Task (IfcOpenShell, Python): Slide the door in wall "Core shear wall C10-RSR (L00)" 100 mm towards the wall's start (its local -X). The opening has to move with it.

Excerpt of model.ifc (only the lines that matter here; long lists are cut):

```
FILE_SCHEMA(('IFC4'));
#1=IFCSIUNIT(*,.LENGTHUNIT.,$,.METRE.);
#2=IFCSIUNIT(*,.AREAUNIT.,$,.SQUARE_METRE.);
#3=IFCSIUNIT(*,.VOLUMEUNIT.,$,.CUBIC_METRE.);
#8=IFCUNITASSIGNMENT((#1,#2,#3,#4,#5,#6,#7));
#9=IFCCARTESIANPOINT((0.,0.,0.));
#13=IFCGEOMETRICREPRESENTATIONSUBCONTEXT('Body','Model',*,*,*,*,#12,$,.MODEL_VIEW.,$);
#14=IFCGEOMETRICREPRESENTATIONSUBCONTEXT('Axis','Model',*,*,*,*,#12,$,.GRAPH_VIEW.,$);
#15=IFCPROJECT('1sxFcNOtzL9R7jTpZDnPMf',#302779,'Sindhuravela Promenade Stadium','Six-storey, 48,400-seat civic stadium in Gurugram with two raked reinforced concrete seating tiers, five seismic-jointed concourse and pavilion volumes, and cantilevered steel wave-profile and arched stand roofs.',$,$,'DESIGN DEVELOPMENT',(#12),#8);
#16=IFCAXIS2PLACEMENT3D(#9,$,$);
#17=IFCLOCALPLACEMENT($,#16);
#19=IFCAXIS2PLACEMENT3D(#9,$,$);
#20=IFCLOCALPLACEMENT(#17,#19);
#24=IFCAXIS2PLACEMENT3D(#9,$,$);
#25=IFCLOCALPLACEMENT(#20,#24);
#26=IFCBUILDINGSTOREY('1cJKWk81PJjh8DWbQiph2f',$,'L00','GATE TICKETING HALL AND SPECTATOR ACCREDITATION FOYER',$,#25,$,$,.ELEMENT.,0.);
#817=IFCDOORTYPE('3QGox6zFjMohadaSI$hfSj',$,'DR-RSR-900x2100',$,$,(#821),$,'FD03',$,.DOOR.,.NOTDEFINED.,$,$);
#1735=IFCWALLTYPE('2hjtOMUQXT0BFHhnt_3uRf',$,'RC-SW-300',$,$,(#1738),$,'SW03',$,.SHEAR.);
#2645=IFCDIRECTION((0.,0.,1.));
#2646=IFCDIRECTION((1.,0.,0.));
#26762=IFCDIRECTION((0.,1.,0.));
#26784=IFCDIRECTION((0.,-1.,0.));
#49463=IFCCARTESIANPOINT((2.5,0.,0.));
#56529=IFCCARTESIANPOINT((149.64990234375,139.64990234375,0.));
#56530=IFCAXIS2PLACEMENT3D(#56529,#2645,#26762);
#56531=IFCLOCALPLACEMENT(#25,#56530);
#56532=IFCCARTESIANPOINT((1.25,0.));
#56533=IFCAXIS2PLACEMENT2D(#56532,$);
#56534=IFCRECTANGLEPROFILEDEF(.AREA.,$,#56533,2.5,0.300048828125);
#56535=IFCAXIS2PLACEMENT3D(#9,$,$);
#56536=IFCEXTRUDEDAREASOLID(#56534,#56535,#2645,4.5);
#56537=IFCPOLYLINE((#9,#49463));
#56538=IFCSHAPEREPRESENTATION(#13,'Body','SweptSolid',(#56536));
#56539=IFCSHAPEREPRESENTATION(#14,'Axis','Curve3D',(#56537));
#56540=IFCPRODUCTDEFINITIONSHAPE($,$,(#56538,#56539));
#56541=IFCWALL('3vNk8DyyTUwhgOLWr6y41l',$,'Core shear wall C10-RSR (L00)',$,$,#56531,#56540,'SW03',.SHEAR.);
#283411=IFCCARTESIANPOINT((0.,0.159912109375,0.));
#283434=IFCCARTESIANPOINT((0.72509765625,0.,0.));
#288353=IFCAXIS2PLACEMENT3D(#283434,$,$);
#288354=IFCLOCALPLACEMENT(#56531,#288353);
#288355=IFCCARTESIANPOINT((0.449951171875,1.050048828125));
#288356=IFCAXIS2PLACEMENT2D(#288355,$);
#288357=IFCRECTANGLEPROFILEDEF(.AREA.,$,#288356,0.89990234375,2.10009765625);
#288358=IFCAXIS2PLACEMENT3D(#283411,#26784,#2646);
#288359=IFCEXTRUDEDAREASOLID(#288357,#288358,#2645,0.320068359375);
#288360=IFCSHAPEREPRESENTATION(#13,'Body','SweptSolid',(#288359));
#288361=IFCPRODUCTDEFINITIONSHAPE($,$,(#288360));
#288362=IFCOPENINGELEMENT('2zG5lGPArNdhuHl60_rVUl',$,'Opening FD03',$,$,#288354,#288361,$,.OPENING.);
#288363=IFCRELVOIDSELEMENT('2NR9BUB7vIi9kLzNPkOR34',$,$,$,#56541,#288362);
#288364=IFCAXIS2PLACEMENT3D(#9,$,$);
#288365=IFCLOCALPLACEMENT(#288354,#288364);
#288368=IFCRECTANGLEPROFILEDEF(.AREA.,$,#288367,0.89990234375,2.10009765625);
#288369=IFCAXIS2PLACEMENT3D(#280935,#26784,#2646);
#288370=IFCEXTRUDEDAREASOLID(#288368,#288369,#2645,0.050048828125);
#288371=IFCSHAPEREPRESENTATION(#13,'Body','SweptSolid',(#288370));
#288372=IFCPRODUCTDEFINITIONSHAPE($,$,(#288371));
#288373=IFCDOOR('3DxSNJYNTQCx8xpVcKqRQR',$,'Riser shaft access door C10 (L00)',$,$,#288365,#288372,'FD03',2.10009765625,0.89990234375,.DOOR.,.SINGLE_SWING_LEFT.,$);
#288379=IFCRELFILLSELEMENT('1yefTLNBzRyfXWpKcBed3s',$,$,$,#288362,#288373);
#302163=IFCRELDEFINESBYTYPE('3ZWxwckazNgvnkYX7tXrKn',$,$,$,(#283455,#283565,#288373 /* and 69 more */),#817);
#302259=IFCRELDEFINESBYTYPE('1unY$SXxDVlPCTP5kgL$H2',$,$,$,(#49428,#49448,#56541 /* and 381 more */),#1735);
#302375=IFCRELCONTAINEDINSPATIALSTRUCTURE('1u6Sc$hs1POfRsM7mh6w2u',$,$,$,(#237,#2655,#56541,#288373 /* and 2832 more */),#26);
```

```python
import ifcopenshell
import ifcopenshell.api.geometry
import ifcopenshell.util.placement
import ifcopenshell.util.unit

model = ifcopenshell.open("model.ifc")
unit_scale = ifcopenshell.util.unit.calculate_unit_scale(model)

door = model.by_guid("3DxSNJYNTQCx8xpVcKqRQR")
opening = door.FillsVoids[0].RelatingOpeningElement
wall = opening.VoidsElements[0].RelatingBuildingElement

wall_matrix = ifcopenshell.util.placement.get_local_placement(wall.ObjectPlacement)
shift = wall_matrix[:3, 0] * -0.1 / unit_scale
before = ifcopenshell.util.placement.get_local_placement(door.ObjectPlacement)[:3, 3].copy()

# The door is placed relative to its opening, so it follows when the opening moves.
matrix = ifcopenshell.util.placement.get_local_placement(opening.ObjectPlacement)
matrix[:3, 3] += shift
ifcopenshell.api.geometry.edit_object_placement(
    model, product=opening, matrix=matrix, is_si=False, should_transform_children=True
)

after = ifcopenshell.util.placement.get_local_placement(door.ObjectPlacement)[:3, 3]
print("door moved by", (after - before).round(3) + 0.0)

model.write("model_rev.ifc")
```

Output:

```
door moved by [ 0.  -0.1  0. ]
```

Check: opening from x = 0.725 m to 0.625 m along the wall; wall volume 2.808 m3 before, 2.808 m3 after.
